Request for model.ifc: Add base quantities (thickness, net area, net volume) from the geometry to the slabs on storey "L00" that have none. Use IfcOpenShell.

First a look at what the model holds.

```python
import ifcopenshell
import ifcopenshell.util.element
import ifcopenshell.util.unit

model = ifcopenshell.open("model.ifc")
print(model.schema)
for unit_type in ("LENGTHUNIT", "AREAUNIT", "VOLUMEUNIT"):
    print(unit_type, ifcopenshell.util.unit.calculate_unit_scale(model, unit_type))
storey = next(s for s in model.by_type("IfcBuildingStorey") if s.Name == "L00")
slabs = [e for e in ifcopenshell.util.element.get_decomposition(storey) if e.is_a("IfcSlab")]
for e in sorted(slabs, key=lambda e: e.id()):
    print(e.id(), e.is_a(), e.Name, list(ifcopenshell.util.element.get_psets(e, qtos_only=True)), sep=" | ")
```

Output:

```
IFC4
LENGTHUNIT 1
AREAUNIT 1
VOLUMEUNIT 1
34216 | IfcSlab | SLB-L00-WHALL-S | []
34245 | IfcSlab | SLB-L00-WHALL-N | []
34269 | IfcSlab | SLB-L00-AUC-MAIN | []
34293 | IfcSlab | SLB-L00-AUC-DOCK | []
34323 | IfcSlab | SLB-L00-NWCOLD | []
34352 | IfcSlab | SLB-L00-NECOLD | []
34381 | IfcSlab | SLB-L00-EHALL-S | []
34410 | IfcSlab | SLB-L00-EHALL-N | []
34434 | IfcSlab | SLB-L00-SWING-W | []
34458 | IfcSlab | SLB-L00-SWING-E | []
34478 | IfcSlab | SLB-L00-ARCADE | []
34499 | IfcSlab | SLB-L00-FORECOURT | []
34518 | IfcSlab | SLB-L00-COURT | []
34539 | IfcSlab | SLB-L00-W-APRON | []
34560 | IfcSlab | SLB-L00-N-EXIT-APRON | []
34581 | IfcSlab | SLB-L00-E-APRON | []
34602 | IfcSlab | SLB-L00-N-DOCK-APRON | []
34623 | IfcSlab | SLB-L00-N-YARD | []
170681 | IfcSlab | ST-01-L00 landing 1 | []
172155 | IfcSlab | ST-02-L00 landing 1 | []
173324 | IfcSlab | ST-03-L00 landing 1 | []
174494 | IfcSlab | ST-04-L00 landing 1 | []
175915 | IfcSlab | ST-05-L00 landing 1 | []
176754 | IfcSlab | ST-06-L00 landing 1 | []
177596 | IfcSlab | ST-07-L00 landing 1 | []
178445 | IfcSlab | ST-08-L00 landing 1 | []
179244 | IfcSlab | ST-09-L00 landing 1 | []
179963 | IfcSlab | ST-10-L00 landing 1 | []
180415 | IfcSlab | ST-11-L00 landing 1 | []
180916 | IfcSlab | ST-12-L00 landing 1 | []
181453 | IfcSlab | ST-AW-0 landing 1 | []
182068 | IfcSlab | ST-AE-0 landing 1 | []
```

```python
import ifcopenshell
import ifcopenshell.api.pset
import ifcopenshell.geom
import ifcopenshell.util.element
import ifcopenshell.util.shape
import ifcopenshell.util.unit

model = ifcopenshell.open("model.ifc")
unit_scale = ifcopenshell.util.unit.calculate_unit_scale(model)
area_scale = ifcopenshell.util.unit.calculate_unit_scale(model, "AREAUNIT")
volume_scale = ifcopenshell.util.unit.calculate_unit_scale(model, "VOLUMEUNIT")
settings = ifcopenshell.geom.settings()

storey = next(s for s in model.by_type("IfcBuildingStorey") if s.Name == "L00")
slabs = [e for e in ifcopenshell.util.element.get_decomposition(storey) if e.is_a("IfcSlab")]

for e in sorted(slabs, key=lambda e: e.id()):
    if ifcopenshell.util.element.get_psets(e, qtos_only=True, should_inherit=False):
        continue
    # Geometry comes back in metres, in the element's own axes.
    shape = ifcopenshell.geom.create_shape(settings, e)
    values = {
        "Width": ifcopenshell.util.shape.get_z(shape.geometry) / unit_scale,
        "NetArea": ifcopenshell.util.shape.get_footprint_area(shape.geometry) / area_scale,
        "NetVolume": ifcopenshell.util.shape.get_volume(shape.geometry) / volume_scale,
    }
    qto = ifcopenshell.api.pset.add_qto(model, product=e, name="Qto_SlabBaseQuantities")
    ifcopenshell.api.pset.edit_qto(model, qto=qto, properties=values)
    print(e.id(), {k: round(v, 3) for k, v in values.items()})

model.write("model-out.ifc")
```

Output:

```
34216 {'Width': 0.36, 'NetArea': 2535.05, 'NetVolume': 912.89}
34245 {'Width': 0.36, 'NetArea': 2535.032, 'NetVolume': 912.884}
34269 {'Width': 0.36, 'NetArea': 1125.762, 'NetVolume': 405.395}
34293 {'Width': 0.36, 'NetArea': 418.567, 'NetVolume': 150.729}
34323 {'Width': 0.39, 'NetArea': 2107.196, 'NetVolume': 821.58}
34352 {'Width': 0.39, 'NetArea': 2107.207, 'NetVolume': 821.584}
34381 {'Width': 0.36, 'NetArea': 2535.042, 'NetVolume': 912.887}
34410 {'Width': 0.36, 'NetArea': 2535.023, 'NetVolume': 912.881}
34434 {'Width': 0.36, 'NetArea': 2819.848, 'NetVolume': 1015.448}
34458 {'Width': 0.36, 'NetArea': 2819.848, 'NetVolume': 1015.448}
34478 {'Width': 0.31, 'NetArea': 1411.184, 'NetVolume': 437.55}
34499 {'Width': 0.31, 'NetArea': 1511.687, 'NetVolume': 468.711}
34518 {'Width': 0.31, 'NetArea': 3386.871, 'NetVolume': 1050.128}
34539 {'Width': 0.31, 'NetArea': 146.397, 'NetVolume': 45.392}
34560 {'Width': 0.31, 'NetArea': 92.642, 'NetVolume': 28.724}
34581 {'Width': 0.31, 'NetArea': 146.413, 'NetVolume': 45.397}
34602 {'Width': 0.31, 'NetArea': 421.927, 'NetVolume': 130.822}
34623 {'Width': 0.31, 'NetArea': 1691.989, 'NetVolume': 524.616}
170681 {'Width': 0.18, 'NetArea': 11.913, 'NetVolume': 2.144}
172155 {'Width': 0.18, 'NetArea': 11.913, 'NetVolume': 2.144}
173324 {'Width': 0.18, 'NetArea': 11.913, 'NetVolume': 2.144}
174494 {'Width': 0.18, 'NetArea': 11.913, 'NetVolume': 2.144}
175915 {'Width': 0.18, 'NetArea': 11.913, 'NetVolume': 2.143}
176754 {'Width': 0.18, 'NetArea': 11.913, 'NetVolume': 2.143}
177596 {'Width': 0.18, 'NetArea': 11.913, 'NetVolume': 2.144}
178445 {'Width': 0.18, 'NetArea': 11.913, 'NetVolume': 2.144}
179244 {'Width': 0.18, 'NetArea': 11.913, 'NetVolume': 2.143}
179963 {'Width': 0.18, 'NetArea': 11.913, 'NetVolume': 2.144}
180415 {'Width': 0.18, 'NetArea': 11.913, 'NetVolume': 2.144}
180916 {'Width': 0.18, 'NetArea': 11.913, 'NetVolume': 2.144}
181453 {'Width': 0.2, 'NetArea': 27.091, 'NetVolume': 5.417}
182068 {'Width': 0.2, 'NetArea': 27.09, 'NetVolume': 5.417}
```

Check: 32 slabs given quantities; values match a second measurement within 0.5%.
